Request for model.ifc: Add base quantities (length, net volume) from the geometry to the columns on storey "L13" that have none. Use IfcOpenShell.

First a look at what the model holds.

```python
import ifcopenshell
import ifcopenshell.util.element
import ifcopenshell.util.unit

model = ifcopenshell.open("model.ifc")
print(model.schema)
for unit_type in ("LENGTHUNIT", "AREAUNIT", "VOLUMEUNIT"):
    print(unit_type, ifcopenshell.util.unit.calculate_unit_scale(model, unit_type))
storey = next(s for s in model.by_type("IfcBuildingStorey") if s.Name == "L13")
columns = [e for e in ifcopenshell.util.element.get_decomposition(storey) if e.is_a("IfcColumn")]
for e in sorted(columns, key=lambda e: e.id()):
    print(e.id(), e.is_a(), e.Name, list(ifcopenshell.util.element.get_psets(e, qtos_only=True)), sep=" | ")
```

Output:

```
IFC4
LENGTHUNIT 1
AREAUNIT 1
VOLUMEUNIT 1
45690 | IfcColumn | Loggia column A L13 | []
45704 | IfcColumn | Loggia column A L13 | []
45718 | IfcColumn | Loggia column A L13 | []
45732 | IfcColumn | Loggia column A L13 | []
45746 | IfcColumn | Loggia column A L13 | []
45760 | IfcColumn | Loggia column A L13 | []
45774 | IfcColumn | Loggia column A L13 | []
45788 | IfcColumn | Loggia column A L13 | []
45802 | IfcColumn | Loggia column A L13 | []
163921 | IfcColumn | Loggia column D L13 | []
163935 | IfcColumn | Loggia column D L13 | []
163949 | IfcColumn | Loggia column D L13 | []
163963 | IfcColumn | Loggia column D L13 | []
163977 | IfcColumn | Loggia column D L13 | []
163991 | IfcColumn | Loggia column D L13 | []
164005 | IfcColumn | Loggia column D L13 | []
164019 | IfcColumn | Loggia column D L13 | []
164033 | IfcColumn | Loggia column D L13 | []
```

```python
import ifcopenshell
import ifcopenshell.api.pset
import ifcopenshell.geom
import ifcopenshell.util.element
import ifcopenshell.util.shape
import ifcopenshell.util.unit

model = ifcopenshell.open("model.ifc")
unit_scale = ifcopenshell.util.unit.calculate_unit_scale(model)
volume_scale = ifcopenshell.util.unit.calculate_unit_scale(model, "VOLUMEUNIT")
settings = ifcopenshell.geom.settings()

storey = next(s for s in model.by_type("IfcBuildingStorey") if s.Name == "L13")
columns = [e for e in ifcopenshell.util.element.get_decomposition(storey) if e.is_a("IfcColumn")]

for e in sorted(columns, key=lambda e: e.id()):
    if ifcopenshell.util.element.get_psets(e, qtos_only=True, should_inherit=False):
        continue
    # Geometry comes back in metres, in the element's own axes.
    shape = ifcopenshell.geom.create_shape(settings, e)
    values = {
        "Length": ifcopenshell.util.shape.get_z(shape.geometry) / unit_scale,
        "NetVolume": ifcopenshell.util.shape.get_volume(shape.geometry) / volume_scale,
    }
    qto = ifcopenshell.api.pset.add_qto(model, product=e, name="Qto_ColumnBaseQuantities")
    ifcopenshell.api.pset.edit_qto(model, qto=qto, properties=values)
    print(e.id(), {k: round(v, 3) for k, v in values.items()})

model.write("model-out.ifc")
```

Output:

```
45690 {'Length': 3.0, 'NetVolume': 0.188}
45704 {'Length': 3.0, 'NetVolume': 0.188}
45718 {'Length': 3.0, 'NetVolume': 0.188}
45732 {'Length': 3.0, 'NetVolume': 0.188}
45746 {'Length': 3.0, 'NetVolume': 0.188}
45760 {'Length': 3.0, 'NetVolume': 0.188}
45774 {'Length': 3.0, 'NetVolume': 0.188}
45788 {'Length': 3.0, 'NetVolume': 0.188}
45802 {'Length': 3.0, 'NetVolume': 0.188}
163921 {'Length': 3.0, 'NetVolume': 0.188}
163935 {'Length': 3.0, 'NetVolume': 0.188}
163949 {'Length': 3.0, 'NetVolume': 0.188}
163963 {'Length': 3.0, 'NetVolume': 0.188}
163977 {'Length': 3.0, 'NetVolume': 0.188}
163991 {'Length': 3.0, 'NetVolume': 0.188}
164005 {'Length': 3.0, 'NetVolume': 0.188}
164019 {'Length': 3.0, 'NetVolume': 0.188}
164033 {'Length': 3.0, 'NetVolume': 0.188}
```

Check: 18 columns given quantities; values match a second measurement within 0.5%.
